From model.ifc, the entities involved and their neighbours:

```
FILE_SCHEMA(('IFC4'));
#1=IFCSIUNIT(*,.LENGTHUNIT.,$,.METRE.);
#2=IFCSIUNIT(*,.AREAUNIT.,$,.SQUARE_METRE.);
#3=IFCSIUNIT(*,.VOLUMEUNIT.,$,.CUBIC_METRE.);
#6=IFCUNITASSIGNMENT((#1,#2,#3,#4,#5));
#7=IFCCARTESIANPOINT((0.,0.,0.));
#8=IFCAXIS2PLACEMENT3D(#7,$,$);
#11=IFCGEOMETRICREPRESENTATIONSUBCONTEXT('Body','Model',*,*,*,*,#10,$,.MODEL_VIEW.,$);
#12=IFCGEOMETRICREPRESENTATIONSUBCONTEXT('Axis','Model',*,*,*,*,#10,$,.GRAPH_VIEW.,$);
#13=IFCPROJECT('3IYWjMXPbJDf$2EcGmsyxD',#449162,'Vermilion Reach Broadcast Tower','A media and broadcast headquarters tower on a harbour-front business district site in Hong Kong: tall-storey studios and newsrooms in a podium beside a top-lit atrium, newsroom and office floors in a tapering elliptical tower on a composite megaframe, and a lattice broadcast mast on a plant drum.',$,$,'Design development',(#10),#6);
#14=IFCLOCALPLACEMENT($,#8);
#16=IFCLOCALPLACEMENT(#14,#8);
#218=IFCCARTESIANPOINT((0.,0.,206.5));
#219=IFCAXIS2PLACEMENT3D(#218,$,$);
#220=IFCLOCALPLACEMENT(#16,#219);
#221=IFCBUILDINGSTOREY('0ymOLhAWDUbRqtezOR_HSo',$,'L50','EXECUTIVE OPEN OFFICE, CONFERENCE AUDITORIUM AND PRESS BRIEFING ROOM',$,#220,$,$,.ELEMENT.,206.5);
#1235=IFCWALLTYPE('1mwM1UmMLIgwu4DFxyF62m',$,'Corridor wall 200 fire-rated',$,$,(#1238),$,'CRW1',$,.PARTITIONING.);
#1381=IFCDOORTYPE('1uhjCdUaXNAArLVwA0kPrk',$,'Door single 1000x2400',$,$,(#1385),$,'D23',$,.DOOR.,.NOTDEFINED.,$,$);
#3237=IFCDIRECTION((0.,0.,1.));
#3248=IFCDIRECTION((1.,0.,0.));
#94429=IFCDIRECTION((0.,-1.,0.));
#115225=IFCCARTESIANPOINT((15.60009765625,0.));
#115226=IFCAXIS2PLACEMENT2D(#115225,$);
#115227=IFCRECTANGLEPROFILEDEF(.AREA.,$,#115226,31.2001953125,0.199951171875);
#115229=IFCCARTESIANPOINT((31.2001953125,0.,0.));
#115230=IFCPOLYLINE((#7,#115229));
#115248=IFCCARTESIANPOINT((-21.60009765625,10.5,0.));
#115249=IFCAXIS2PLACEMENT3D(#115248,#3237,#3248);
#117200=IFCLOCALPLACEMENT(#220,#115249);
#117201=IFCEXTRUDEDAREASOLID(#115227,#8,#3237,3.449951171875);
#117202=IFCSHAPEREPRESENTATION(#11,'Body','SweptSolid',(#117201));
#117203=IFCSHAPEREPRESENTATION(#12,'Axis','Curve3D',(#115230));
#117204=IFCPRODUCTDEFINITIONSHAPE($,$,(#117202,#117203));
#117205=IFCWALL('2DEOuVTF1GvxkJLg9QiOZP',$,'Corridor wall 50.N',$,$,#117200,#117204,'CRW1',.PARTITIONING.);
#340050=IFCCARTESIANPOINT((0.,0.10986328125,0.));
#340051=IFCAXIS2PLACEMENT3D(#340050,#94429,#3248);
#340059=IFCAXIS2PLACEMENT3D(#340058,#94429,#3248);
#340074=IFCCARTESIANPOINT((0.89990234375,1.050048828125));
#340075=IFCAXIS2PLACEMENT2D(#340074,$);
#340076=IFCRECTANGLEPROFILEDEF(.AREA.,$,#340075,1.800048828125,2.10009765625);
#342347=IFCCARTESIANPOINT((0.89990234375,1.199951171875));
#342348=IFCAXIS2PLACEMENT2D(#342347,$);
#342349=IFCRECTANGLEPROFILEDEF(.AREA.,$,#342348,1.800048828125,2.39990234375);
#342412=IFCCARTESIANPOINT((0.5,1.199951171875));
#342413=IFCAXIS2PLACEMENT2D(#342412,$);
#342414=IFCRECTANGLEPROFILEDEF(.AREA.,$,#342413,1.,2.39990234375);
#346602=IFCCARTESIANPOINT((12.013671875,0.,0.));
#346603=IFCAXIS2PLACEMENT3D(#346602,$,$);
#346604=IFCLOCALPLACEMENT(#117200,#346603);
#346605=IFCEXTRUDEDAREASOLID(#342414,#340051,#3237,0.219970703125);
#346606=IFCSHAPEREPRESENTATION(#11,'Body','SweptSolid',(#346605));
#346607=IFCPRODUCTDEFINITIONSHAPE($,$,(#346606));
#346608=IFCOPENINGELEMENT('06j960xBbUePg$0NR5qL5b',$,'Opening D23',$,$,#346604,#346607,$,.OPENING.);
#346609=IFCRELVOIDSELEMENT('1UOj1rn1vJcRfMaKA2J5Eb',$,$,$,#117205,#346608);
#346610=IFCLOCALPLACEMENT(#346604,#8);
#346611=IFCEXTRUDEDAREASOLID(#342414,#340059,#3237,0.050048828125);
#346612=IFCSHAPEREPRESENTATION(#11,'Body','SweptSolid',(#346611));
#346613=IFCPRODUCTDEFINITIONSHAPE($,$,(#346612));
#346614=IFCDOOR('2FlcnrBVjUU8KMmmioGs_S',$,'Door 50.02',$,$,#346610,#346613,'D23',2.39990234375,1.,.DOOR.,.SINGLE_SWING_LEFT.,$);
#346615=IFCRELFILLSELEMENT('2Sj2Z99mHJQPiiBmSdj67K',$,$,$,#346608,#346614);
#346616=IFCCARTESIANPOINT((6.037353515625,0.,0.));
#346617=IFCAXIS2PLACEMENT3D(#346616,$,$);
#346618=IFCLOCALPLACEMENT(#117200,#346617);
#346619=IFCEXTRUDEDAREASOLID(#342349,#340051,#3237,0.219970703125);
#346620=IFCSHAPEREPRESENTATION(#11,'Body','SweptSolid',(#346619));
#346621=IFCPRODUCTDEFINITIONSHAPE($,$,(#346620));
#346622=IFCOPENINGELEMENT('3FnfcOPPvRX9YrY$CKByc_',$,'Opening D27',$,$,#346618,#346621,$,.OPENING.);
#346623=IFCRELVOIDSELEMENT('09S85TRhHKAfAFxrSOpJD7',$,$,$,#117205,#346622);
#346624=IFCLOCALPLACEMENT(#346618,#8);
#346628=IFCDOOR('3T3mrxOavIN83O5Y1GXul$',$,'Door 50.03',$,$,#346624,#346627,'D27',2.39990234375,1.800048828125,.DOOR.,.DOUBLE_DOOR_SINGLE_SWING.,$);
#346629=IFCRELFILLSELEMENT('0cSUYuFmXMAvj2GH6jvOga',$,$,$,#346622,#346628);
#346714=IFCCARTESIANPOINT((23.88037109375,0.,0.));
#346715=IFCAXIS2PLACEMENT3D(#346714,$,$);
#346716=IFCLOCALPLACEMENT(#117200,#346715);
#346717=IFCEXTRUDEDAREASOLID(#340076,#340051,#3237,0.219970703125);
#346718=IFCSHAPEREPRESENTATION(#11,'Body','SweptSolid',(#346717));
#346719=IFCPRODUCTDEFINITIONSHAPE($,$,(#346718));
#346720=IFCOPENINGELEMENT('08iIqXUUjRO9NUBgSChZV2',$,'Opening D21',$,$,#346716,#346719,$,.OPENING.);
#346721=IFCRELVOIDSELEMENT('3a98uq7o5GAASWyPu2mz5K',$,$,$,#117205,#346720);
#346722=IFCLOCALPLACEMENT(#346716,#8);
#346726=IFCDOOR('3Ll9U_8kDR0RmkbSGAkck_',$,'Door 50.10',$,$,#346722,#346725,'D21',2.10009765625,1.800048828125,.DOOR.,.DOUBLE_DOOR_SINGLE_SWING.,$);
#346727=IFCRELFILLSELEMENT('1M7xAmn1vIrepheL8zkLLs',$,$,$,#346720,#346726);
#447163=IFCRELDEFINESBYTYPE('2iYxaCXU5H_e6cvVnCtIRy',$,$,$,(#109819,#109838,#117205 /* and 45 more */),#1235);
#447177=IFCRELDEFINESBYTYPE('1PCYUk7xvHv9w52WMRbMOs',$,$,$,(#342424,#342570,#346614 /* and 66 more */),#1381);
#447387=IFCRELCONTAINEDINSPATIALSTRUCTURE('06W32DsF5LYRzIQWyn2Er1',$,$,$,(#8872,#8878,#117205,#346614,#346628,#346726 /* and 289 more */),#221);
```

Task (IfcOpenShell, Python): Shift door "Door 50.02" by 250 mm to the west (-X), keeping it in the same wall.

```python
import ifcopenshell
import ifcopenshell.api.geometry
import ifcopenshell.util.placement

model = ifcopenshell.open("model.ifc")

door = model.by_guid("2FlcnrBVjUU8KMmmioGs_S")
opening = door.FillsVoids[0].RelatingOpeningElement
wall = opening.VoidsElements[0].RelatingBuildingElement

wall_matrix = ifcopenshell.util.placement.get_local_placement(wall.ObjectPlacement)
shift = wall_matrix[:3, 0] * -0.25
before = ifcopenshell.util.placement.get_local_placement(door.ObjectPlacement)[:3, 3].copy()

# The door is placed relative to its opening, so it follows when the opening moves.
matrix = ifcopenshell.util.placement.get_local_placement(opening.ObjectPlacement)
matrix[:3, 3] += shift
ifcopenshell.api.geometry.edit_object_placement(
    model, product=opening, matrix=matrix, is_si=False, should_transform_children=True
)

after = ifcopenshell.util.placement.get_local_placement(door.ObjectPlacement)[:3, 3]
print("door moved by", (after - before).round(3) + 0.0)

model.write("model_rev.ifc")
```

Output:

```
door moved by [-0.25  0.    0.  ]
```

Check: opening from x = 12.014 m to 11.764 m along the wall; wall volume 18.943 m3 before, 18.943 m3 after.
